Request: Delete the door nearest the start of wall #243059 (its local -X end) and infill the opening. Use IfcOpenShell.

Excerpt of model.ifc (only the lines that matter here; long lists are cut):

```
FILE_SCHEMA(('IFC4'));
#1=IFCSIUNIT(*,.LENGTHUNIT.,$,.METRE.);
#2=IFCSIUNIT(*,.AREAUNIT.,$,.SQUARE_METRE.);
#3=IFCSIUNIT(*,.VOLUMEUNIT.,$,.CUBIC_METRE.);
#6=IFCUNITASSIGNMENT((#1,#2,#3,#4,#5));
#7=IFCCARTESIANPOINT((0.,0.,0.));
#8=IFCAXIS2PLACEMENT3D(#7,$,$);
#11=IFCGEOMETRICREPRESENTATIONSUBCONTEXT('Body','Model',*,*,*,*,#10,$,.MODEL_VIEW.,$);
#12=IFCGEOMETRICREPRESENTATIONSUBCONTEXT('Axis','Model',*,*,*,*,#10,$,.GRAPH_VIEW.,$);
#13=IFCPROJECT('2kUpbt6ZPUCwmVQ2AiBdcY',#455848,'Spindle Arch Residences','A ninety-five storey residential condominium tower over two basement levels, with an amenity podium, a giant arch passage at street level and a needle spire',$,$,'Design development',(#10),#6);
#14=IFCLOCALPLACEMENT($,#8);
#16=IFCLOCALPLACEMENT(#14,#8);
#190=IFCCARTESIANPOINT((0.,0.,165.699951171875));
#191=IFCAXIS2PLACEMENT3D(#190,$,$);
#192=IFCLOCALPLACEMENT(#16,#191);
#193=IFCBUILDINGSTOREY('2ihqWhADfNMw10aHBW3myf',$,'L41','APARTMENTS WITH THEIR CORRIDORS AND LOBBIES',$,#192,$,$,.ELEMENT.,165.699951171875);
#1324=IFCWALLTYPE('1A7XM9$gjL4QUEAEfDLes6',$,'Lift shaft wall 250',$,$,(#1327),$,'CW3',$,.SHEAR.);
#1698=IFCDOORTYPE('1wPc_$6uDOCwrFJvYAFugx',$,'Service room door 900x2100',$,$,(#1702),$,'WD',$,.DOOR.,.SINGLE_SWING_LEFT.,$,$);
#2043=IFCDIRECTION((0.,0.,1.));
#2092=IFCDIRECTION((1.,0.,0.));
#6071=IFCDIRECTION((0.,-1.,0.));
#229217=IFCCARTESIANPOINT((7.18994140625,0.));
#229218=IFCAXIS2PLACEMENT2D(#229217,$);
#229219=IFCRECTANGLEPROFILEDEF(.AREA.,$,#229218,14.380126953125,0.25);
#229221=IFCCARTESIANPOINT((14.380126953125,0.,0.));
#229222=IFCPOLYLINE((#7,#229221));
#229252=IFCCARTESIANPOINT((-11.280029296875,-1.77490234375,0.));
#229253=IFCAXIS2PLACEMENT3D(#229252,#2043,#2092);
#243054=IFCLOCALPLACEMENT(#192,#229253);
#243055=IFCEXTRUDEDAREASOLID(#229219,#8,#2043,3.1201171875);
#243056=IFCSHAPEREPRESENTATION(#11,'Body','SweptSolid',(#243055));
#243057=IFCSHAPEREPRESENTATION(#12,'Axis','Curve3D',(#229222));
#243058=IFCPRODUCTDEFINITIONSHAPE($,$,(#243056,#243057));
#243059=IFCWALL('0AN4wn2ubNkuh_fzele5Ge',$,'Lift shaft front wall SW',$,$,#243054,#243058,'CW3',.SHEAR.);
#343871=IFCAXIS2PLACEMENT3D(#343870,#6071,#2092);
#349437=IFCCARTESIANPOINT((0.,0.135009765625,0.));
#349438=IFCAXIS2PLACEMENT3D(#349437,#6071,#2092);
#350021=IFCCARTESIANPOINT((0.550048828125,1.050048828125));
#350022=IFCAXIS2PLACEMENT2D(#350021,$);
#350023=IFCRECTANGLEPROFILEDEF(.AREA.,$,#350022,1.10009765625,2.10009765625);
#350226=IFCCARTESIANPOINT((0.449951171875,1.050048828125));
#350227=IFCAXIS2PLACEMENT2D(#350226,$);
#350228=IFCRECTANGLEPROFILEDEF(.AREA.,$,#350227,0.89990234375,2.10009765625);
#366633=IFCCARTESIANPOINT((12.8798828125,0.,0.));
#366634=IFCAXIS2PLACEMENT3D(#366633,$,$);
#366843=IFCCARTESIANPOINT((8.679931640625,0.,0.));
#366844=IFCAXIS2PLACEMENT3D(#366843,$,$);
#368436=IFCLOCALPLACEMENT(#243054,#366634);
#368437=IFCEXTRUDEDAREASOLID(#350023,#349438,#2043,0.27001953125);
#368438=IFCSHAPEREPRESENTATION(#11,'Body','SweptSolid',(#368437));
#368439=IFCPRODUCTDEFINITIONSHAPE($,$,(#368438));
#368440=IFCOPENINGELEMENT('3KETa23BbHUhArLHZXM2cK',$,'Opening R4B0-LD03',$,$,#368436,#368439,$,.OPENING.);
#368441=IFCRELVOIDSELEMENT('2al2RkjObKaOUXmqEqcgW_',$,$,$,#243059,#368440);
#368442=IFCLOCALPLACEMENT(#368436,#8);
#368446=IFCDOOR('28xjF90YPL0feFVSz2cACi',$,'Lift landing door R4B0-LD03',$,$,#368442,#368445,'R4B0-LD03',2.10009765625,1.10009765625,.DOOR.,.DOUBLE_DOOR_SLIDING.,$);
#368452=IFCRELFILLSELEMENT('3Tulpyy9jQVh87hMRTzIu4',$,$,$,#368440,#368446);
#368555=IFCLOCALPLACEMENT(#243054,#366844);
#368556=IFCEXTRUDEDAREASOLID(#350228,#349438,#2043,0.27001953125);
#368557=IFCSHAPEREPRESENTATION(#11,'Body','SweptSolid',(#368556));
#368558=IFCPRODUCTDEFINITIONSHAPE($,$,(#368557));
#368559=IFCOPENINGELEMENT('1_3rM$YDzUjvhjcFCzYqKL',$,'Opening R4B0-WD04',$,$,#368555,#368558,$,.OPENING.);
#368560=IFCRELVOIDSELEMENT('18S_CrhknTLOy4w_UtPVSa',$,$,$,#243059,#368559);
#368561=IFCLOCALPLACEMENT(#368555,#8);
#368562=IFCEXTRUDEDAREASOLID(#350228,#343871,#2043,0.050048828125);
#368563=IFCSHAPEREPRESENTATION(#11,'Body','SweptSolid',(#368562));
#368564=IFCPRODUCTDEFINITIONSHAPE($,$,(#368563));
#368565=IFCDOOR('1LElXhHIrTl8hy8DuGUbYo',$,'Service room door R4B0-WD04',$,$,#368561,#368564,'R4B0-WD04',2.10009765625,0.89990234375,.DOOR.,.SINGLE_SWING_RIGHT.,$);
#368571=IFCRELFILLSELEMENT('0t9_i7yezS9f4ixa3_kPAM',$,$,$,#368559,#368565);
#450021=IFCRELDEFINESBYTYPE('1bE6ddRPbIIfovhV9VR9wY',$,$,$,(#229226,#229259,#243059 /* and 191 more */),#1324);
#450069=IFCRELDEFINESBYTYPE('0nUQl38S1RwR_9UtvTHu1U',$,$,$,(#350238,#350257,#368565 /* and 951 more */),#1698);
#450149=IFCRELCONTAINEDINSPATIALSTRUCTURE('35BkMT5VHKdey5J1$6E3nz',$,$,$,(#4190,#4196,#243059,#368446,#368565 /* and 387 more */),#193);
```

```python
import ifcopenshell
import ifcopenshell.api.feature
import ifcopenshell.api.root
import ifcopenshell.geom
import ifcopenshell.util.shape

model = ifcopenshell.open("model.ifc")
settings = ifcopenshell.geom.settings()


def volume(element):
    """Net volume in cubic metres, openings subtracted."""
    shape = ifcopenshell.geom.create_shape(settings, element)
    return ifcopenshell.util.shape.get_volume(shape.geometry)


door = model.by_guid("1LElXhHIrTl8hy8DuGUbYo")
opening = door.FillsVoids[0].RelatingOpeningElement
wall = opening.VoidsElements[0].RelatingBuildingElement
before = volume(wall)

ifcopenshell.api.root.remove_product(model, product=door)
ifcopenshell.api.feature.remove_feature(model, feature=opening)

after = volume(wall)

print(f"wall volume {before:.3f} -> {after:.3f} m3")

model.write("model-out.ifc")
```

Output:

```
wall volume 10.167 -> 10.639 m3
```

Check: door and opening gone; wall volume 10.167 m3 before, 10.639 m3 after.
